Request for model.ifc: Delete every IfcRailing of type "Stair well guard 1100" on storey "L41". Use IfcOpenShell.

First a look at what the model holds.

```python
import ifcopenshell
import ifcopenshell.util.element

model = ifcopenshell.open("model.ifc")
print(model.schema)
storey = next(s for s in model.by_type("IfcBuildingStorey") if s.Name == "L41")
railings = [e for e in ifcopenshell.util.element.get_decomposition(storey) if e.is_a("IfcRailing")]
seen = {}
for e in railings:
    element_type = ifcopenshell.util.element.get_type(e)
    name = element_type.Name if element_type not in (None, e) else None
    seen[name] = seen.get(name, 0) + 1
for name, count in sorted(seen.items(), key=str):
    print(count, "x", name)
```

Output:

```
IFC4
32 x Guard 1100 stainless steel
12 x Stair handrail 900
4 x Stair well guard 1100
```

```python
import ifcopenshell
import ifcopenshell.api.root
import ifcopenshell.util.element

model = ifcopenshell.open("model.ifc")

storey = next(s for s in model.by_type("IfcBuildingStorey") if s.Name == "L41")
railings = [e for e in ifcopenshell.util.element.get_decomposition(storey) if e.is_a("IfcRailing")]
targets = [e for e in railings if (t := ifcopenshell.util.element.get_type(e)) not in (None, e) and t.Name == "Stair well guard 1100"]

for e in targets:
    ifcopenshell.api.root.remove_product(model, product=e)
print(len(targets), "removed")

model.write("model_edited.ifc")
```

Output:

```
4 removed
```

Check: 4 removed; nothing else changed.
